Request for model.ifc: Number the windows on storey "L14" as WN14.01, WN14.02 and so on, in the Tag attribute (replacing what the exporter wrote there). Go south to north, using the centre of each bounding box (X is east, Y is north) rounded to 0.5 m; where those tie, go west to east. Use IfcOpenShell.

First a look at what the model holds.

```python
import ifcopenshell
import ifcopenshell.util.element
import ifcopenshell.util.placement

model = ifcopenshell.open("model.ifc")
print(model.schema)
storey = next(s for s in model.by_type("IfcBuildingStorey") if s.Name == "L14")
windows = [e for e in ifcopenshell.util.element.get_decomposition(storey) if e.is_a("IfcWindow")]
for e in sorted(windows, key=lambda e: e.id()):
    origin = ifcopenshell.util.placement.get_local_placement(e.ObjectPlacement)[:3, 3]
    print(e.id(), e.Tag, e.Name, origin.round(2) + 0.0, sep=" | ")
```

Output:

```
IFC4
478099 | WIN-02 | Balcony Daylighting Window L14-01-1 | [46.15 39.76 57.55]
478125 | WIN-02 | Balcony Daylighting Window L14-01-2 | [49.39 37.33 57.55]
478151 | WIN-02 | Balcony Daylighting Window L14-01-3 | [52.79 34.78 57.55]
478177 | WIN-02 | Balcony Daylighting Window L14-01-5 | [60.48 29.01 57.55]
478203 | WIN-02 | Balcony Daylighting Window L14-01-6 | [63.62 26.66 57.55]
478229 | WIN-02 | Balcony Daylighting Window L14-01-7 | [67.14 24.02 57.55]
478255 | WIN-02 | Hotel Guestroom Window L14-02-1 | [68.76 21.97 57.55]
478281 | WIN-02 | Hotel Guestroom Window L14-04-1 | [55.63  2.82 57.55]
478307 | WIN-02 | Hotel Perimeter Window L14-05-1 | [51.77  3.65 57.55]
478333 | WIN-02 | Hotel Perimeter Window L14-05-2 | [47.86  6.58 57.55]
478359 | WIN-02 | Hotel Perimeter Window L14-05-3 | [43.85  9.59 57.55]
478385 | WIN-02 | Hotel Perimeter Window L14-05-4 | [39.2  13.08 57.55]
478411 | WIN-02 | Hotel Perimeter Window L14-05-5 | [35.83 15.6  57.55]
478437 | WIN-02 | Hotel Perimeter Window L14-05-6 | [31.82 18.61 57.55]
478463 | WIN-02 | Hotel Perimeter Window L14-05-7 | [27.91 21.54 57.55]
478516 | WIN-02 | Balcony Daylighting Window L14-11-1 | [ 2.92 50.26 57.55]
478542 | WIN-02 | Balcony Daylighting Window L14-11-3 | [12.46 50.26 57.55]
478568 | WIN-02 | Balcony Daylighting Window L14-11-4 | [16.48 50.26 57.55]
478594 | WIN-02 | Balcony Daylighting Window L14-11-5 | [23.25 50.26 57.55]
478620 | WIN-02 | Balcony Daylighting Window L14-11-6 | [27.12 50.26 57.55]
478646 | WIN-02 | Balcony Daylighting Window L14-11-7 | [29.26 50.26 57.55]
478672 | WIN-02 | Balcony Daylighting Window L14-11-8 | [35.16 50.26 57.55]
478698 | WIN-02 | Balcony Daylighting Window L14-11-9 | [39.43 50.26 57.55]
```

```python
import ifcopenshell
import ifcopenshell.geom
import ifcopenshell.util.element
import ifcopenshell.util.shape

model = ifcopenshell.open("model.ifc")
settings = ifcopenshell.geom.settings()
settings.set("use-world-coords", True)


def centre(element):
    shape = ifcopenshell.geom.create_shape(settings, element)
    return ifcopenshell.util.shape.get_bbox_centroid(shape.geometry)


storey = next(s for s in model.by_type("IfcBuildingStorey") if s.Name == "L14")
windows = [e for e in ifcopenshell.util.element.get_decomposition(storey) if e.is_a("IfcWindow")]

# Insertion points can sit at a corner or the storey origin, so sort by the geometry (in metres).
centres = {e: centre(e) for e in windows}
windows.sort(key=lambda e: (round(centres[e][1] / 0.5), centres[e][0]))

for i, e in enumerate(windows, start=1):
    number = f"WN14.{i:02d}"
    e.Tag = number
    print(e.id(), number)

model.write("model_rev.ifc")
```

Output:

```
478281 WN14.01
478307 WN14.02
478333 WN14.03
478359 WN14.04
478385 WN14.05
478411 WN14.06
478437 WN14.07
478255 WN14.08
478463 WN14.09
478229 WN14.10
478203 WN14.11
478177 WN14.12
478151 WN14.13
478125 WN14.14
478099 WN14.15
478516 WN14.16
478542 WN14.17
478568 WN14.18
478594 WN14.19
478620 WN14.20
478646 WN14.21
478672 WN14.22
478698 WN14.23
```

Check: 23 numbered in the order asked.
